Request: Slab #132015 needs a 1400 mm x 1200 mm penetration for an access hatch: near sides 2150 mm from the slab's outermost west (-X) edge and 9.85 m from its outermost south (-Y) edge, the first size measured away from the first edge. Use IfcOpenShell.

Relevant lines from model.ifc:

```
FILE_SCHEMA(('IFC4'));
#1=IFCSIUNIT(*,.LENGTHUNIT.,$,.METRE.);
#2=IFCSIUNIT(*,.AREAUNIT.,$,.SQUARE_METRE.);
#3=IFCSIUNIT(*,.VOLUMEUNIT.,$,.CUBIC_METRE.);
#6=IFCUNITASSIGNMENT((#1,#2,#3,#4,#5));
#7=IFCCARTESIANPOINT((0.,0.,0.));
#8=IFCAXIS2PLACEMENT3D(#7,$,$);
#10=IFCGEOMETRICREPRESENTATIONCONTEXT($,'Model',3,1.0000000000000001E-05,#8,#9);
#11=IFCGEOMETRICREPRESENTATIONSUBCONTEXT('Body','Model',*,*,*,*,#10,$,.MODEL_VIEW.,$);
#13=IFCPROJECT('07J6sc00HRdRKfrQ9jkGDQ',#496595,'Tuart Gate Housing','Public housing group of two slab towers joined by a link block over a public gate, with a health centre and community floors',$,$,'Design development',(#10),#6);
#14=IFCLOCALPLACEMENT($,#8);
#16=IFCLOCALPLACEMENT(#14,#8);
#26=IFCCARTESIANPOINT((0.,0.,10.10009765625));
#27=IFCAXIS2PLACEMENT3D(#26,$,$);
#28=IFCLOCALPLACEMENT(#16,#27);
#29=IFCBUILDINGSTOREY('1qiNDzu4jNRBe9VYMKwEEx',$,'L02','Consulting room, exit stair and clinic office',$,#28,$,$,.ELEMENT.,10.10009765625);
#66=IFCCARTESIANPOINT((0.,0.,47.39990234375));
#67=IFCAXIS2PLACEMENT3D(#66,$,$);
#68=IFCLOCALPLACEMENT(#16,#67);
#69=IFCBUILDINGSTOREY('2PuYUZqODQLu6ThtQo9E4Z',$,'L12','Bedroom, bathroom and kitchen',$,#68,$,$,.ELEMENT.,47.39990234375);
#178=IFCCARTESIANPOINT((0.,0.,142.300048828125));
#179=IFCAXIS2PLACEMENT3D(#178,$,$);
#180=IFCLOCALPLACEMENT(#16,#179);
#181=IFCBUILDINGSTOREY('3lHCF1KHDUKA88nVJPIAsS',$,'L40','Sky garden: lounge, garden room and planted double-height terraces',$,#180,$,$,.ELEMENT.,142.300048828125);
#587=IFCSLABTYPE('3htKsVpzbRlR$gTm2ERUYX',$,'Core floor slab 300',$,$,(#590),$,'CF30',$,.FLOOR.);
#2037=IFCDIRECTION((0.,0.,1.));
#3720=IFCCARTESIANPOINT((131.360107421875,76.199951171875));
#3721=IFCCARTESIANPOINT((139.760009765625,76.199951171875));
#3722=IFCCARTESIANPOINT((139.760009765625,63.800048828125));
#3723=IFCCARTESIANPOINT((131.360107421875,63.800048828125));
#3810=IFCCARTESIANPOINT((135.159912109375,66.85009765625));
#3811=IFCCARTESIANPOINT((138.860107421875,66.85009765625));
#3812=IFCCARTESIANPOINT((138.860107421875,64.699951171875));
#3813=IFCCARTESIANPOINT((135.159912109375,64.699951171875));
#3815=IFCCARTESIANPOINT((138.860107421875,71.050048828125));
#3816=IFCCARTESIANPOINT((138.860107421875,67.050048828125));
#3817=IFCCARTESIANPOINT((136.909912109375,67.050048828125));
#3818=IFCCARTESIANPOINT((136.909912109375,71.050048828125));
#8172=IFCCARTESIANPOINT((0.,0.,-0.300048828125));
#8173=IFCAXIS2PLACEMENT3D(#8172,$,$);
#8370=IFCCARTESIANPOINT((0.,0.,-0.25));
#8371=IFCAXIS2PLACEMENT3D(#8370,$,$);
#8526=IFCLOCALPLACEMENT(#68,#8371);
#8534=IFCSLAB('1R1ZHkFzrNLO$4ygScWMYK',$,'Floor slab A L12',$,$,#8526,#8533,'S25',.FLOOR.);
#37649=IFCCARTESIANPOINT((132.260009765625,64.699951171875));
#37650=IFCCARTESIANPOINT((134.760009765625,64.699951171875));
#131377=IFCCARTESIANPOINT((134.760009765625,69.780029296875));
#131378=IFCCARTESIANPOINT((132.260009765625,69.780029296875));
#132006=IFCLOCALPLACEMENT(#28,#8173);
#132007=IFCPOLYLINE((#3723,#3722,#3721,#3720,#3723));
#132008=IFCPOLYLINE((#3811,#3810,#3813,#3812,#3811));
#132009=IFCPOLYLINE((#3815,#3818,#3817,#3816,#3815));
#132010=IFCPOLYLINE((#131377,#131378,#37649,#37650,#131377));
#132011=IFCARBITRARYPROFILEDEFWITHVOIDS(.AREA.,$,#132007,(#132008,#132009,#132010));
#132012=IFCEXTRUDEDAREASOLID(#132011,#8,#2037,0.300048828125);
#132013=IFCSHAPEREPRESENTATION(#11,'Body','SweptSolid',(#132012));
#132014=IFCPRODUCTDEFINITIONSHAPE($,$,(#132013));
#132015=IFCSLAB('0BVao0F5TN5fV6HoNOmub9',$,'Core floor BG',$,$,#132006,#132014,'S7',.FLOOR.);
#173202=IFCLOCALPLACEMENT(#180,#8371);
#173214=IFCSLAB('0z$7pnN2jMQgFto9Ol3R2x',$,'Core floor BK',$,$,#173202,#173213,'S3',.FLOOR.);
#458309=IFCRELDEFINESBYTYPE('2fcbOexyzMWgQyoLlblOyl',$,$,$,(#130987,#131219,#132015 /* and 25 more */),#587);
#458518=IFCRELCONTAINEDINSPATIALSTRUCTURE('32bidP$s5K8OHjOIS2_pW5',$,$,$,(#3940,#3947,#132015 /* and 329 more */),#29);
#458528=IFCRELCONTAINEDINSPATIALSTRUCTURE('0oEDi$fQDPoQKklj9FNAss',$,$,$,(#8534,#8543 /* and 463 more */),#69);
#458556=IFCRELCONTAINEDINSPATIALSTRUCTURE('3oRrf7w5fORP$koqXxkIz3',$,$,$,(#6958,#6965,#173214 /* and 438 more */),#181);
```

```python
import numpy as np
import ifcopenshell
import ifcopenshell.api.feature
import ifcopenshell.api.geometry
import ifcopenshell.api.root
import ifcopenshell.geom
import ifcopenshell.util.placement
import ifcopenshell.util.representation
import ifcopenshell.util.shape
import ifcopenshell.util.unit

model = ifcopenshell.open("model.ifc")
unit_scale = ifcopenshell.util.unit.calculate_unit_scale(model)
settings = ifcopenshell.geom.settings()


def volume(element):
    """Net volume in cubic metres, openings subtracted."""
    shape = ifcopenshell.geom.create_shape(settings, element)
    return ifcopenshell.util.shape.get_volume(shape.geometry)


slab = model.by_guid("0BVao0F5TN5fV6HoNOmub9")
before = volume(slab)

# Extent in the slab's own axes, in metres. The edges named are its -X and -Y sides.
slab_shape = ifcopenshell.geom.create_shape(settings, slab)
vertices = ifcopenshell.util.shape.get_vertices(slab_shape.geometry)
x_min, y_min, bottom = vertices.min(axis=0)
top = vertices[:, 2].max()

opening = ifcopenshell.api.root.create_entity(model, ifc_class="IfcOpeningElement", name="Access hatch opening", predefined_type="OPENING")
context = ifcopenshell.util.representation.get_context(model, "Model", "Body", "MODEL_VIEW")
width, depth = 1.4, 1.2
outline = [(0.0, 0.0), (width, 0.0), (width, depth), (0.0, depth), (0.0, 0.0)]
# Overshoot both faces by 50 mm so the cut is clean.
shape = ifcopenshell.api.geometry.add_slab_representation(
    model, context=context, depth=top - bottom + 0.1, polyline=outline
)
ifcopenshell.api.geometry.assign_representation(model, product=opening, representation=shape)

matrix = ifcopenshell.util.placement.get_local_placement(slab.ObjectPlacement)
matrix[:, 3] = matrix @ np.append(np.array([x_min + 2.15, y_min + 9.85, bottom - 0.05]) / unit_scale, 1.0)
ifcopenshell.api.geometry.edit_object_placement(model, product=opening, matrix=matrix, is_si=False)
ifcopenshell.api.feature.add_feature(model, feature=opening, element=slab)

after = volume(slab)

print(f"slab volume {before:.3f} -> {after:.3f} m3")

model.write("model_rev.ifc")
```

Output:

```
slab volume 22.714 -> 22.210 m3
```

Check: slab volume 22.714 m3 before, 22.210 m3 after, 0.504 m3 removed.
